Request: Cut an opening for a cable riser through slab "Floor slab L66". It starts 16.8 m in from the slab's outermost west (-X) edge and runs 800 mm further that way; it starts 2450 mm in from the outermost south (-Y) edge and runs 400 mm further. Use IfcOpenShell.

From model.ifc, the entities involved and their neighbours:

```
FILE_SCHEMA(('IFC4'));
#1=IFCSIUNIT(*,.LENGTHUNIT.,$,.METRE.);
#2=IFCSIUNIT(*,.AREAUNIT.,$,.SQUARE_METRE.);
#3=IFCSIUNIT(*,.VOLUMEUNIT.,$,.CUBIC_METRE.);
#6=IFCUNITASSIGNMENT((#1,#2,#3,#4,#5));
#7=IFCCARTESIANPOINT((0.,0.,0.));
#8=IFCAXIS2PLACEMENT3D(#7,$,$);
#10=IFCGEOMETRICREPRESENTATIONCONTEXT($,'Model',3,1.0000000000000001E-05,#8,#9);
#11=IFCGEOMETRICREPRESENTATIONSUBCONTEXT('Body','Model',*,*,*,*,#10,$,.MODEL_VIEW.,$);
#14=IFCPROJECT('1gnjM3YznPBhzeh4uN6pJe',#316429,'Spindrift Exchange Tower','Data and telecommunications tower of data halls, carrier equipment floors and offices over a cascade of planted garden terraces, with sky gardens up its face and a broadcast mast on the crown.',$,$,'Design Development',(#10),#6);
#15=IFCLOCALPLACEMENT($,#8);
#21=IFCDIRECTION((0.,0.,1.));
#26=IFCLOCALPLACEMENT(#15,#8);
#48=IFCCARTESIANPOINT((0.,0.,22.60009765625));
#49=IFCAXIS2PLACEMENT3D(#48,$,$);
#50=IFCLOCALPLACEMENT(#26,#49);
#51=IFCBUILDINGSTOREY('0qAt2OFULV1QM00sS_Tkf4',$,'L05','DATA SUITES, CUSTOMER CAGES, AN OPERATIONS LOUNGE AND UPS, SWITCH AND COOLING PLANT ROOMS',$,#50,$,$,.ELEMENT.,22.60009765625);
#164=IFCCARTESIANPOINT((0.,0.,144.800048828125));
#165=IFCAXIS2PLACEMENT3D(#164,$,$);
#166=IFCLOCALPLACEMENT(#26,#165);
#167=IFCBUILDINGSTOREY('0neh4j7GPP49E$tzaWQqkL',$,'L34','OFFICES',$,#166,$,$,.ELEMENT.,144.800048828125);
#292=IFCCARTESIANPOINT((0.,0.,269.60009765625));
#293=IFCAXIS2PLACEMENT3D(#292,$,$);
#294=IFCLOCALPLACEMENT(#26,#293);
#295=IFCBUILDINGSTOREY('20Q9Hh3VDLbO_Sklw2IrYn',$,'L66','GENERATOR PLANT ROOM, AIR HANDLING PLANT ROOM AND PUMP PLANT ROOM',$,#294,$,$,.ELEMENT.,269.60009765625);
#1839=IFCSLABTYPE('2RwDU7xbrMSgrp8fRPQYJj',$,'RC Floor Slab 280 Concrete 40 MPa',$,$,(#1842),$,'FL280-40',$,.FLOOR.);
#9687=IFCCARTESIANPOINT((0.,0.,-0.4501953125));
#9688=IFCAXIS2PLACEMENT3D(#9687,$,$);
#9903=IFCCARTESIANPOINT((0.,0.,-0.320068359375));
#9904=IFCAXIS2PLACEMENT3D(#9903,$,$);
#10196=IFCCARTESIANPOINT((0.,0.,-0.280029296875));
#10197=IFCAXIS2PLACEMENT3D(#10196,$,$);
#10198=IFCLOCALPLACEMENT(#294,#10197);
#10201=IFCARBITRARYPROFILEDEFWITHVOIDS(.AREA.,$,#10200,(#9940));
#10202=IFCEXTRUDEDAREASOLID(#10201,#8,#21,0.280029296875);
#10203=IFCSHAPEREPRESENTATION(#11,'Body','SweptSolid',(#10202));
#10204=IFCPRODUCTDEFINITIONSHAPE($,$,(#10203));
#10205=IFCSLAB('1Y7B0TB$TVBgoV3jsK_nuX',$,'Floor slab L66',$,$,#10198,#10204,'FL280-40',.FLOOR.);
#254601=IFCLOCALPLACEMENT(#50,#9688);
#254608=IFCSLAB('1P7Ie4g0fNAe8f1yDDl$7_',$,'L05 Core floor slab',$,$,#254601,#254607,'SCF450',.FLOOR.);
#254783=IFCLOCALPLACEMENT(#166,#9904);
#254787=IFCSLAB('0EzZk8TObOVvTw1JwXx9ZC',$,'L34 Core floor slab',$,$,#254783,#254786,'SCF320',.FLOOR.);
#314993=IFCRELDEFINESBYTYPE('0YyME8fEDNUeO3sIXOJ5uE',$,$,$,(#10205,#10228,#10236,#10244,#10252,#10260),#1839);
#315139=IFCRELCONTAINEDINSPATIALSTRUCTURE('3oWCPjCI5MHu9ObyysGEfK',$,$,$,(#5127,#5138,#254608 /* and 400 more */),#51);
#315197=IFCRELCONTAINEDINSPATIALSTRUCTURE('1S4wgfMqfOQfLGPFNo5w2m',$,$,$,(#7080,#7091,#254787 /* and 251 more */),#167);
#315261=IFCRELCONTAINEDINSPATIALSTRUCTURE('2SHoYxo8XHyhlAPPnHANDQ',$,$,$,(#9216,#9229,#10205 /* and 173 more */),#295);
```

```python
import numpy as np
import ifcopenshell
import ifcopenshell.api.feature
import ifcopenshell.api.geometry
import ifcopenshell.api.root
import ifcopenshell.geom
import ifcopenshell.util.placement
import ifcopenshell.util.representation
import ifcopenshell.util.shape
import ifcopenshell.util.unit

model = ifcopenshell.open("model.ifc")
unit_scale = ifcopenshell.util.unit.calculate_unit_scale(model)
settings = ifcopenshell.geom.settings()


def volume(element):
    """Net volume in cubic metres, openings subtracted."""
    shape = ifcopenshell.geom.create_shape(settings, element)
    return ifcopenshell.util.shape.get_volume(shape.geometry)


slab = model.by_id(10205)
before = volume(slab)

# Extent in the slab's own axes, in metres. The edges named are its -X and -Y sides.
slab_shape = ifcopenshell.geom.create_shape(settings, slab)
vertices = ifcopenshell.util.shape.get_vertices(slab_shape.geometry)
x_min, y_min, bottom = vertices.min(axis=0)
top = vertices[:, 2].max()

opening = ifcopenshell.api.root.create_entity(model, ifc_class="IfcOpeningElement", name="Cable riser opening", predefined_type="OPENING")
context = ifcopenshell.util.representation.get_context(model, "Model", "Body", "MODEL_VIEW")
width, depth = 0.8, 0.4
outline = [(0.0, 0.0), (width, 0.0), (width, depth), (0.0, depth), (0.0, 0.0)]
# Overshoot both faces by 50 mm so the cut is clean.
shape = ifcopenshell.api.geometry.add_slab_representation(
    model, context=context, depth=top - bottom + 0.1, polyline=outline
)
ifcopenshell.api.geometry.assign_representation(model, product=opening, representation=shape)

matrix = ifcopenshell.util.placement.get_local_placement(slab.ObjectPlacement)
matrix[:, 3] = matrix @ np.append(np.array([x_min + 16.8, y_min + 2.45, bottom - 0.05]) / unit_scale, 1.0)
ifcopenshell.api.geometry.edit_object_placement(model, product=opening, matrix=matrix, is_si=False)
ifcopenshell.api.feature.add_feature(model, feature=opening, element=slab)

after = volume(slab)

print(f"slab volume {before:.3f} -> {after:.3f} m3")

model.write("model-out.ifc")
```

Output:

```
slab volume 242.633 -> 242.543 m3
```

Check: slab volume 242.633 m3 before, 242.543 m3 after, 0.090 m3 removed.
